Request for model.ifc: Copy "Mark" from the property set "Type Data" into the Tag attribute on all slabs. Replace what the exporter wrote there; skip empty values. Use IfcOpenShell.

First a look at what the model holds.

```python
import ifcopenshell
import ifcopenshell.util.element

model = ifcopenshell.open("model.ifc")
print(model.schema)
slabs = model.by_type("IfcSlab")
print(len(slabs), "slabs")
for e in slabs[:8]:
    source = ifcopenshell.util.element.get_pset(e, "Type Data", "Mark")
    target = e.Tag
    print(e.id(), repr(source), repr(target), sep=" | ")
```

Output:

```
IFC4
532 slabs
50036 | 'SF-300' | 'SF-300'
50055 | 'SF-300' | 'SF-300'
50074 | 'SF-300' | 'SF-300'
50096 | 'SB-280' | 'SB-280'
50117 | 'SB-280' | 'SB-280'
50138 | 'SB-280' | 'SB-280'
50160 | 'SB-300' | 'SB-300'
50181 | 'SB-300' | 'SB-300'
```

```python
import ifcopenshell
import ifcopenshell.util.element

model = ifcopenshell.open("model.ifc")

count = 0
for e in model.by_type("IfcSlab"):
    value = ifcopenshell.util.element.get_pset(e, "Type Data", "Mark")
    current = e.Tag
    if not value or not value.strip() or current == value:
        continue
    e.Tag = value
    count += 1

print(count, "slabs updated")

model.write("model-out.ifc")
```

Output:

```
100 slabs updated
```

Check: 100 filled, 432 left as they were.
